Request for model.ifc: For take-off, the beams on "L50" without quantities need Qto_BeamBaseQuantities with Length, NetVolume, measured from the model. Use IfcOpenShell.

First a look at what the model holds.

```python
import ifcopenshell
import ifcopenshell.util.element
import ifcopenshell.util.unit

model = ifcopenshell.open("model.ifc")
print(model.schema)
for unit_type in ("LENGTHUNIT", "AREAUNIT", "VOLUMEUNIT"):
    print(unit_type, ifcopenshell.util.unit.calculate_unit_scale(model, unit_type))
storey = next(s for s in model.by_type("IfcBuildingStorey") if s.Name == "L50")
beams = [e for e in ifcopenshell.util.element.get_decomposition(storey) if e.is_a("IfcBeam")]
for e in sorted(beams, key=lambda e: e.id()):
    print(e.id(), e.is_a(), e.Name, list(ifcopenshell.util.element.get_psets(e, qtos_only=True)), sep=" | ")
```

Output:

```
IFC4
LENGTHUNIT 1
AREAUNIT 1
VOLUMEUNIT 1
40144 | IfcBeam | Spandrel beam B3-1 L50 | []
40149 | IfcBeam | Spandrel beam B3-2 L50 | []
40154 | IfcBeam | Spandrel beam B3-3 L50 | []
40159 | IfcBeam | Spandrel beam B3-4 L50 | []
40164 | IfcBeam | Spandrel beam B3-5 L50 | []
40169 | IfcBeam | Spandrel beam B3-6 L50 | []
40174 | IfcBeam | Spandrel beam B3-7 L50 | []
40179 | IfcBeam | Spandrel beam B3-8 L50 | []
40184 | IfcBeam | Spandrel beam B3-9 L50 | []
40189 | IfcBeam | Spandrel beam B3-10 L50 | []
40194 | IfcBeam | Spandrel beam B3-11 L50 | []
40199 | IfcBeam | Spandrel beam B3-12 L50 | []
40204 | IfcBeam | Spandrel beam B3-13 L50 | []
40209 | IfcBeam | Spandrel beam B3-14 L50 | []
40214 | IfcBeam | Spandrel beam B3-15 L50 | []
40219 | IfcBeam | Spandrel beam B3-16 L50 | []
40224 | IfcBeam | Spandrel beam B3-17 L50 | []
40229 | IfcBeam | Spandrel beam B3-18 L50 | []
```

```python
import ifcopenshell
import ifcopenshell.api.pset
import ifcopenshell.geom
import ifcopenshell.util.element
import ifcopenshell.util.shape
import ifcopenshell.util.unit

model = ifcopenshell.open("model.ifc")
unit_scale = ifcopenshell.util.unit.calculate_unit_scale(model)
volume_scale = ifcopenshell.util.unit.calculate_unit_scale(model, "VOLUMEUNIT")
settings = ifcopenshell.geom.settings()

storey = next(s for s in model.by_type("IfcBuildingStorey") if s.Name == "L50")
beams = [e for e in ifcopenshell.util.element.get_decomposition(storey) if e.is_a("IfcBeam")]

for e in sorted(beams, key=lambda e: e.id()):
    if ifcopenshell.util.element.get_psets(e, qtos_only=True, should_inherit=False):
        continue
    # Geometry comes back in metres, in the element's own axes.
    shape = ifcopenshell.geom.create_shape(settings, e)
    values = {
        "Length": ifcopenshell.util.shape.get_max_xyz(shape.geometry) / unit_scale,
        "NetVolume": ifcopenshell.util.shape.get_volume(shape.geometry) / volume_scale,
    }
    qto = ifcopenshell.api.pset.add_qto(model, product=e, name="Qto_BeamBaseQuantities")
    ifcopenshell.api.pset.edit_qto(model, qto=qto, properties=values)
    print(e.id(), {k: round(v, 3) for k, v in values.items()})

model.write("model_rev.ifc")
```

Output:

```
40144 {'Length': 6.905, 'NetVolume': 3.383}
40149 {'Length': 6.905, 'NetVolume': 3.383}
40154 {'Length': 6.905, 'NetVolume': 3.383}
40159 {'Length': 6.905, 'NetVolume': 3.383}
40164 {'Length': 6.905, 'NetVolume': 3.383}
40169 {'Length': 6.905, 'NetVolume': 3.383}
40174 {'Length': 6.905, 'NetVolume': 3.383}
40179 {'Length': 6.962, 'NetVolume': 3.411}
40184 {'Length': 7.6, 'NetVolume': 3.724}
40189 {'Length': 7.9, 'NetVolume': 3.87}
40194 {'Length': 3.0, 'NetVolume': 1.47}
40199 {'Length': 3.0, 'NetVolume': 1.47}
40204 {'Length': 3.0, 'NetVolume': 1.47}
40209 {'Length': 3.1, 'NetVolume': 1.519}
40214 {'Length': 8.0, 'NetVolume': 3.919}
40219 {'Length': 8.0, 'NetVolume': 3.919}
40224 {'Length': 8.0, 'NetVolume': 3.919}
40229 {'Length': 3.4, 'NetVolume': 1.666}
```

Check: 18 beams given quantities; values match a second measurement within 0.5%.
